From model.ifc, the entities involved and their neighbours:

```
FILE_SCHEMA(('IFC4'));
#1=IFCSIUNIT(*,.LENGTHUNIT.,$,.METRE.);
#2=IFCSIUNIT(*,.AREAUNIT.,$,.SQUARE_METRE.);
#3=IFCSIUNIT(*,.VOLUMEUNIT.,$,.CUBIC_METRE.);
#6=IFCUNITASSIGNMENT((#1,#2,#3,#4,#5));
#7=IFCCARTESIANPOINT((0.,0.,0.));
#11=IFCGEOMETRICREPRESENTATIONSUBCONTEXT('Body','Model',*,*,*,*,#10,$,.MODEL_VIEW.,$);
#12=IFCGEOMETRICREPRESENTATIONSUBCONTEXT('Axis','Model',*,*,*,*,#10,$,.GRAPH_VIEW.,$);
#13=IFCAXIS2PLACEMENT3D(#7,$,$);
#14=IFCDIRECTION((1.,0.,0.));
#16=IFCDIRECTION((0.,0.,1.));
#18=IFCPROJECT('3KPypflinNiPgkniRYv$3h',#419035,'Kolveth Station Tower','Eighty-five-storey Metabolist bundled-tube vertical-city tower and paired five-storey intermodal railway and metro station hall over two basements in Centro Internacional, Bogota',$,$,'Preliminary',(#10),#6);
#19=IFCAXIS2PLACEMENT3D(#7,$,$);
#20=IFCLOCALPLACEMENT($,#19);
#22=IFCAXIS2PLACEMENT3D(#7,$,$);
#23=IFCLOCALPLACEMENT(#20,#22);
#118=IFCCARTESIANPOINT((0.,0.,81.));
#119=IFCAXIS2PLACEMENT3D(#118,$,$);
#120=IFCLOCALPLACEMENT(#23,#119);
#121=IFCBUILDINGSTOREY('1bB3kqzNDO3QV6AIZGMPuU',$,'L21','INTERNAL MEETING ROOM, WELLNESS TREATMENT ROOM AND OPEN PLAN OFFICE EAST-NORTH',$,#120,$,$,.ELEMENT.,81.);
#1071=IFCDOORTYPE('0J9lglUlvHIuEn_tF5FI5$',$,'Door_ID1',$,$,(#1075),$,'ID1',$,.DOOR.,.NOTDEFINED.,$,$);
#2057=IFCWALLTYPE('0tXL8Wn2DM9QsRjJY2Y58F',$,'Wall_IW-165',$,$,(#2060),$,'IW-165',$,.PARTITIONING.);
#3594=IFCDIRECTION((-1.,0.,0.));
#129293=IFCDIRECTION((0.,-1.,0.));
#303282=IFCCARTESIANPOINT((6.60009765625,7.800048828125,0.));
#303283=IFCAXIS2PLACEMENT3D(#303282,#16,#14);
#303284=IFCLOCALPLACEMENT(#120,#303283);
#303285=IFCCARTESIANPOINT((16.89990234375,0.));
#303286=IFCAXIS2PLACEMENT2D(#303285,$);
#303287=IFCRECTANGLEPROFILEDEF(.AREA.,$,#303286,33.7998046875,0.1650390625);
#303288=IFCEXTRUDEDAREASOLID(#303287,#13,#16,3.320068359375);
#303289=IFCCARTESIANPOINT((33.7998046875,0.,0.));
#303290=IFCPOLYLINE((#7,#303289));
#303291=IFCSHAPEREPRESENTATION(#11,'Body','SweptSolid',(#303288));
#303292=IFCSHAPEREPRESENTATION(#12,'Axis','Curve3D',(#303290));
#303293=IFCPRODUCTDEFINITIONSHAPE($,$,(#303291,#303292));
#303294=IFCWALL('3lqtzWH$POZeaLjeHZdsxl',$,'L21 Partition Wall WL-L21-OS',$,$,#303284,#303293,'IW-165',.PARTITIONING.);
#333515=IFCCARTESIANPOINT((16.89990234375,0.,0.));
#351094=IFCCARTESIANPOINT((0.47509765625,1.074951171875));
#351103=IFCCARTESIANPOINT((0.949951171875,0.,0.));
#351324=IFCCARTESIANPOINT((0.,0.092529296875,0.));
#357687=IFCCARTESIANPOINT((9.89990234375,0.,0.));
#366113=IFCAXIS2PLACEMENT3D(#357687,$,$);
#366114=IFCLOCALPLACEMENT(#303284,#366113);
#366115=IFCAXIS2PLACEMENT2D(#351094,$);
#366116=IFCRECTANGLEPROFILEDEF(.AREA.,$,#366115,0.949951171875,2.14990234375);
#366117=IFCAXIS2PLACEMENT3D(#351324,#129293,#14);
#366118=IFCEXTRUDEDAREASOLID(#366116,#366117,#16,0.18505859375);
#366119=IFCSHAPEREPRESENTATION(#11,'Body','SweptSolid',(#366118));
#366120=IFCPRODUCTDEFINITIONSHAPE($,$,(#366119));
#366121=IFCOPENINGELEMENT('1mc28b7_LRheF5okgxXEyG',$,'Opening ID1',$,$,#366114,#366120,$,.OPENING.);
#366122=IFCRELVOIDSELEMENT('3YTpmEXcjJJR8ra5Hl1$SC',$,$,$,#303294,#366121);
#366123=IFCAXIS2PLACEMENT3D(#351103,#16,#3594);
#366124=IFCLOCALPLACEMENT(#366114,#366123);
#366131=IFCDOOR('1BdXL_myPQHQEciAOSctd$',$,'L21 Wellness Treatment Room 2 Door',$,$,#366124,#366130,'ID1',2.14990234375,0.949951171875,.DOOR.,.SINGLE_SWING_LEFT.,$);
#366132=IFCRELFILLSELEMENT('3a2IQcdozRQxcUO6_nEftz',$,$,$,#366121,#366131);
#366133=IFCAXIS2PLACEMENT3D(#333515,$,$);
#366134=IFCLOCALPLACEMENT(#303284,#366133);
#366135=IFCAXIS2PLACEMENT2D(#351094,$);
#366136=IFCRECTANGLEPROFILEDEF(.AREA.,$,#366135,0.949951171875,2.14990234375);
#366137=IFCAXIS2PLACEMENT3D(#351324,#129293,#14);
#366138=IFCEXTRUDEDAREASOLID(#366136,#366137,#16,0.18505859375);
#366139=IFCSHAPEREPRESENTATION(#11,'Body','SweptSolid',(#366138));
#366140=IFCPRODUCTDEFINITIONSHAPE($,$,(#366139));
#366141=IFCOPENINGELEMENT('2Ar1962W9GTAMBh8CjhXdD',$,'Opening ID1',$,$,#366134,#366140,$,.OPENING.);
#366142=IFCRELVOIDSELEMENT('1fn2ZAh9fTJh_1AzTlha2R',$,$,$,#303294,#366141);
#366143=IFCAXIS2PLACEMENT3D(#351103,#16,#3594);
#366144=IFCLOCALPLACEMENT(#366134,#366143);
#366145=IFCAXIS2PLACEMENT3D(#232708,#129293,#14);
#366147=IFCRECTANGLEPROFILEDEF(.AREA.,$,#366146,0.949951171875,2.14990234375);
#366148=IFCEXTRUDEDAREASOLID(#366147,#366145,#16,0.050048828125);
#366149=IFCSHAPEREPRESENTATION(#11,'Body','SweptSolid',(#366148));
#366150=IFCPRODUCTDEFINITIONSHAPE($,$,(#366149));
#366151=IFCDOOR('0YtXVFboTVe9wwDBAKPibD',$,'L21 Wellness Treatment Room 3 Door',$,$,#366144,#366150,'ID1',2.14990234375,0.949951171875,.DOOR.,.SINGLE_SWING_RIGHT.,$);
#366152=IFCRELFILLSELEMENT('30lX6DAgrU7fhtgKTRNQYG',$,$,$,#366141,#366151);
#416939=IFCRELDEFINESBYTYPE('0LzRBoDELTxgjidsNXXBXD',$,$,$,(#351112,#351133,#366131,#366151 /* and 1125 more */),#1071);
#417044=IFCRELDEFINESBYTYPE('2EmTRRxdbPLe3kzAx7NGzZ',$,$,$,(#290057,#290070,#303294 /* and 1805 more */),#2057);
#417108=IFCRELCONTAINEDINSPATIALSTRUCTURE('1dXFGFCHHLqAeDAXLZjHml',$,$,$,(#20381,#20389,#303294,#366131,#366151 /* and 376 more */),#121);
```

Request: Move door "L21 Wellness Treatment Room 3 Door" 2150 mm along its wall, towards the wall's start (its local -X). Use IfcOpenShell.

```python
import ifcopenshell
import ifcopenshell.api.geometry
import ifcopenshell.util.placement
import ifcopenshell.util.unit

model = ifcopenshell.open("model.ifc")
unit_scale = ifcopenshell.util.unit.calculate_unit_scale(model)

door = model.by_guid("0YtXVFboTVe9wwDBAKPibD")
opening = door.FillsVoids[0].RelatingOpeningElement
wall = opening.VoidsElements[0].RelatingBuildingElement

wall_matrix = ifcopenshell.util.placement.get_local_placement(wall.ObjectPlacement)
shift = wall_matrix[:3, 0] * -2.15 / unit_scale
before = ifcopenshell.util.placement.get_local_placement(door.ObjectPlacement)[:3, 3].copy()

# The door is placed relative to its opening, so it follows when the opening moves.
matrix = ifcopenshell.util.placement.get_local_placement(opening.ObjectPlacement)
matrix[:3, 3] += shift
ifcopenshell.api.geometry.edit_object_placement(
    model, product=opening, matrix=matrix, is_si=False, should_transform_children=True
)

after = ifcopenshell.util.placement.get_local_placement(door.ObjectPlacement)[:3, 3]
print("door moved by", (after - before).round(3) + 0.0)

model.write("model_rev.ifc")
```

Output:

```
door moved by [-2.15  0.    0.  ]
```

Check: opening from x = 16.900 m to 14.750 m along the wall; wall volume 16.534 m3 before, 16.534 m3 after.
